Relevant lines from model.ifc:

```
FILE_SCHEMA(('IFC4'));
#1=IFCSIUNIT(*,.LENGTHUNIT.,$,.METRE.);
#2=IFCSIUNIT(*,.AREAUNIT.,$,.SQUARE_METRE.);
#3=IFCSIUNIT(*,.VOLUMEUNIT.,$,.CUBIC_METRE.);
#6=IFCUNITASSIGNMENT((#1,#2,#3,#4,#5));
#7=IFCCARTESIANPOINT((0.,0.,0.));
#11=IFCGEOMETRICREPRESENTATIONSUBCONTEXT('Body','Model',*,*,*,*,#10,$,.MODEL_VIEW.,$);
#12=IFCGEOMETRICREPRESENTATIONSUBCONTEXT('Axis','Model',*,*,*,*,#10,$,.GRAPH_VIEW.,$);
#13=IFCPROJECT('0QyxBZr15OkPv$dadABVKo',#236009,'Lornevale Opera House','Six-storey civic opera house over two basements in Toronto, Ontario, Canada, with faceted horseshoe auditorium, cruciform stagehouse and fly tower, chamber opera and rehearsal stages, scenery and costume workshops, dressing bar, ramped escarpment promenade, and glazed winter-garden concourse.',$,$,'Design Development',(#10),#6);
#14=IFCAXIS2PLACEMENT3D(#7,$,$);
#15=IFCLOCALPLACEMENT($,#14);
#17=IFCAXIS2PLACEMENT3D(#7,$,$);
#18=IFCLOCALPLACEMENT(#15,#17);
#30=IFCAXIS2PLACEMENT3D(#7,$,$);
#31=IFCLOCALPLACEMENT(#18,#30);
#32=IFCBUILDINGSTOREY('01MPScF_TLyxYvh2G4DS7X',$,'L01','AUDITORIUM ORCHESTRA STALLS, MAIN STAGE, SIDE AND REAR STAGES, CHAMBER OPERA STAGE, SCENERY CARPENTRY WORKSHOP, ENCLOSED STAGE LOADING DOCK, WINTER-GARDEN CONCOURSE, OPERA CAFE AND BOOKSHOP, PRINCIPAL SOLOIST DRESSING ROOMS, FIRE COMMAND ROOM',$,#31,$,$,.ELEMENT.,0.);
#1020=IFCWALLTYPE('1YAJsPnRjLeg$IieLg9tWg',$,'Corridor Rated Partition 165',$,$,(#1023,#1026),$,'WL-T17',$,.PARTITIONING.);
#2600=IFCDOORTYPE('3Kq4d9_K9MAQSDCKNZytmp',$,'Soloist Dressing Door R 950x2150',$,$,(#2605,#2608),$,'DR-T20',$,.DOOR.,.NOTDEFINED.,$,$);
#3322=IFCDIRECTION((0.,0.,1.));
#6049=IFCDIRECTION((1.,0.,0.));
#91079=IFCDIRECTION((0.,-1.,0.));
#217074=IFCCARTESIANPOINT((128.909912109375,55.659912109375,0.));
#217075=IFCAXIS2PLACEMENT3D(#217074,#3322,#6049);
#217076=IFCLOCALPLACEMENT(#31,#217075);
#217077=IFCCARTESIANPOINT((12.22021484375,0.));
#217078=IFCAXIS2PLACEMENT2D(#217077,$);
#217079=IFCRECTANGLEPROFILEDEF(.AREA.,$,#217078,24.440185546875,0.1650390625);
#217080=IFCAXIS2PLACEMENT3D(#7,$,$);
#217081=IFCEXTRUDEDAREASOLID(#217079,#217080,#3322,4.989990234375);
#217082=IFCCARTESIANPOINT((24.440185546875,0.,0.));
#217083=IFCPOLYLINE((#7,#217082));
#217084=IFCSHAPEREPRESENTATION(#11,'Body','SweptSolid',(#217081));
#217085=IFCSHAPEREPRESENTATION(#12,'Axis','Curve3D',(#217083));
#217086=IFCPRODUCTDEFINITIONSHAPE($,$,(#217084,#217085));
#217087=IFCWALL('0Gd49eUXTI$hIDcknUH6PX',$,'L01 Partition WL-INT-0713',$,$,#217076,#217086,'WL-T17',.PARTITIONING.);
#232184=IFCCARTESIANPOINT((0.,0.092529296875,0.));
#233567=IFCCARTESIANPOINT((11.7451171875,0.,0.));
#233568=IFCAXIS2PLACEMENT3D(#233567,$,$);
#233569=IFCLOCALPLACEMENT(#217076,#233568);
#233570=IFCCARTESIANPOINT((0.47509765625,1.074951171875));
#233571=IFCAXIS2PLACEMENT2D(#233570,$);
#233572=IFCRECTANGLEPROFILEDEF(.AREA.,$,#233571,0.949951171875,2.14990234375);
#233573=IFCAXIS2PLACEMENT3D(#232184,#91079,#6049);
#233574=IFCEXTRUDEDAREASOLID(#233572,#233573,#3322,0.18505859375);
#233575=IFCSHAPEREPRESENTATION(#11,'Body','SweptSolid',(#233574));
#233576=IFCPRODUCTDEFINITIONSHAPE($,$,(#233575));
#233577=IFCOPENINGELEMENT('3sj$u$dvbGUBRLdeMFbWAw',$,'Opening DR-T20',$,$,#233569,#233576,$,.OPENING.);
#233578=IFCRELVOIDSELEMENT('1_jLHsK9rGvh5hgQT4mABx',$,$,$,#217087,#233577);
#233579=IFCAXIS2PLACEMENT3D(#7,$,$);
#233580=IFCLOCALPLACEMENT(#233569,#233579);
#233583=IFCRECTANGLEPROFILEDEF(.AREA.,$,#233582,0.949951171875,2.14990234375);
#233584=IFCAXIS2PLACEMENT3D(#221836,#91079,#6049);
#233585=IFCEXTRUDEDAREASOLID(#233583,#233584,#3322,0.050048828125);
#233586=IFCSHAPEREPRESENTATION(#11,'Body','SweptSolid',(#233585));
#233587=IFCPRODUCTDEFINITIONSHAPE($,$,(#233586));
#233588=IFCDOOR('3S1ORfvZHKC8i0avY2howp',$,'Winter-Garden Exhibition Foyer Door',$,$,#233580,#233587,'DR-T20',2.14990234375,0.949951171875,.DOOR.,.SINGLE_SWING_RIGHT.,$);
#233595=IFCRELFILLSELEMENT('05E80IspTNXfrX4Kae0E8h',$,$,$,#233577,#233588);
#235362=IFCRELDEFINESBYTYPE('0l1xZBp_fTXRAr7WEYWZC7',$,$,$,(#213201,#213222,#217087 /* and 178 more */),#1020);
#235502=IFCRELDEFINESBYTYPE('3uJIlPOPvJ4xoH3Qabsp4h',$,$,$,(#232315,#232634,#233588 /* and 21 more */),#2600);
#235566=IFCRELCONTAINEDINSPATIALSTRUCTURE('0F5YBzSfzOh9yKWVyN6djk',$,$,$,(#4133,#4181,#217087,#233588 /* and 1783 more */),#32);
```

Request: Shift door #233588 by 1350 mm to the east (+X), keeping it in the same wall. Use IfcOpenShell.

```python
import ifcopenshell
import ifcopenshell.api.geometry
import ifcopenshell.util.placement
import ifcopenshell.util.unit

model = ifcopenshell.open("model.ifc")
unit_scale = ifcopenshell.util.unit.calculate_unit_scale(model)

door = model.by_guid("3S1ORfvZHKC8i0avY2howp")
opening = door.FillsVoids[0].RelatingOpeningElement
wall = opening.VoidsElements[0].RelatingBuildingElement

wall_matrix = ifcopenshell.util.placement.get_local_placement(wall.ObjectPlacement)
shift = wall_matrix[:3, 0] * 1.35 / unit_scale
before = ifcopenshell.util.placement.get_local_placement(door.ObjectPlacement)[:3, 3].copy()

# The door is placed relative to its opening, so it follows when the opening moves.
matrix = ifcopenshell.util.placement.get_local_placement(opening.ObjectPlacement)
matrix[:3, 3] += shift
ifcopenshell.api.geometry.edit_object_placement(
    model, product=opening, matrix=matrix, is_si=False, should_transform_children=True
)

after = ifcopenshell.util.placement.get_local_placement(door.ObjectPlacement)[:3, 3]
print("door moved by", (after - before).round(3) + 0.0)

model.write("model-out.ifc")
```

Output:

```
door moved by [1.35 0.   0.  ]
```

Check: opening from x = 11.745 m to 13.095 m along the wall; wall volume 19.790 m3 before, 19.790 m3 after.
